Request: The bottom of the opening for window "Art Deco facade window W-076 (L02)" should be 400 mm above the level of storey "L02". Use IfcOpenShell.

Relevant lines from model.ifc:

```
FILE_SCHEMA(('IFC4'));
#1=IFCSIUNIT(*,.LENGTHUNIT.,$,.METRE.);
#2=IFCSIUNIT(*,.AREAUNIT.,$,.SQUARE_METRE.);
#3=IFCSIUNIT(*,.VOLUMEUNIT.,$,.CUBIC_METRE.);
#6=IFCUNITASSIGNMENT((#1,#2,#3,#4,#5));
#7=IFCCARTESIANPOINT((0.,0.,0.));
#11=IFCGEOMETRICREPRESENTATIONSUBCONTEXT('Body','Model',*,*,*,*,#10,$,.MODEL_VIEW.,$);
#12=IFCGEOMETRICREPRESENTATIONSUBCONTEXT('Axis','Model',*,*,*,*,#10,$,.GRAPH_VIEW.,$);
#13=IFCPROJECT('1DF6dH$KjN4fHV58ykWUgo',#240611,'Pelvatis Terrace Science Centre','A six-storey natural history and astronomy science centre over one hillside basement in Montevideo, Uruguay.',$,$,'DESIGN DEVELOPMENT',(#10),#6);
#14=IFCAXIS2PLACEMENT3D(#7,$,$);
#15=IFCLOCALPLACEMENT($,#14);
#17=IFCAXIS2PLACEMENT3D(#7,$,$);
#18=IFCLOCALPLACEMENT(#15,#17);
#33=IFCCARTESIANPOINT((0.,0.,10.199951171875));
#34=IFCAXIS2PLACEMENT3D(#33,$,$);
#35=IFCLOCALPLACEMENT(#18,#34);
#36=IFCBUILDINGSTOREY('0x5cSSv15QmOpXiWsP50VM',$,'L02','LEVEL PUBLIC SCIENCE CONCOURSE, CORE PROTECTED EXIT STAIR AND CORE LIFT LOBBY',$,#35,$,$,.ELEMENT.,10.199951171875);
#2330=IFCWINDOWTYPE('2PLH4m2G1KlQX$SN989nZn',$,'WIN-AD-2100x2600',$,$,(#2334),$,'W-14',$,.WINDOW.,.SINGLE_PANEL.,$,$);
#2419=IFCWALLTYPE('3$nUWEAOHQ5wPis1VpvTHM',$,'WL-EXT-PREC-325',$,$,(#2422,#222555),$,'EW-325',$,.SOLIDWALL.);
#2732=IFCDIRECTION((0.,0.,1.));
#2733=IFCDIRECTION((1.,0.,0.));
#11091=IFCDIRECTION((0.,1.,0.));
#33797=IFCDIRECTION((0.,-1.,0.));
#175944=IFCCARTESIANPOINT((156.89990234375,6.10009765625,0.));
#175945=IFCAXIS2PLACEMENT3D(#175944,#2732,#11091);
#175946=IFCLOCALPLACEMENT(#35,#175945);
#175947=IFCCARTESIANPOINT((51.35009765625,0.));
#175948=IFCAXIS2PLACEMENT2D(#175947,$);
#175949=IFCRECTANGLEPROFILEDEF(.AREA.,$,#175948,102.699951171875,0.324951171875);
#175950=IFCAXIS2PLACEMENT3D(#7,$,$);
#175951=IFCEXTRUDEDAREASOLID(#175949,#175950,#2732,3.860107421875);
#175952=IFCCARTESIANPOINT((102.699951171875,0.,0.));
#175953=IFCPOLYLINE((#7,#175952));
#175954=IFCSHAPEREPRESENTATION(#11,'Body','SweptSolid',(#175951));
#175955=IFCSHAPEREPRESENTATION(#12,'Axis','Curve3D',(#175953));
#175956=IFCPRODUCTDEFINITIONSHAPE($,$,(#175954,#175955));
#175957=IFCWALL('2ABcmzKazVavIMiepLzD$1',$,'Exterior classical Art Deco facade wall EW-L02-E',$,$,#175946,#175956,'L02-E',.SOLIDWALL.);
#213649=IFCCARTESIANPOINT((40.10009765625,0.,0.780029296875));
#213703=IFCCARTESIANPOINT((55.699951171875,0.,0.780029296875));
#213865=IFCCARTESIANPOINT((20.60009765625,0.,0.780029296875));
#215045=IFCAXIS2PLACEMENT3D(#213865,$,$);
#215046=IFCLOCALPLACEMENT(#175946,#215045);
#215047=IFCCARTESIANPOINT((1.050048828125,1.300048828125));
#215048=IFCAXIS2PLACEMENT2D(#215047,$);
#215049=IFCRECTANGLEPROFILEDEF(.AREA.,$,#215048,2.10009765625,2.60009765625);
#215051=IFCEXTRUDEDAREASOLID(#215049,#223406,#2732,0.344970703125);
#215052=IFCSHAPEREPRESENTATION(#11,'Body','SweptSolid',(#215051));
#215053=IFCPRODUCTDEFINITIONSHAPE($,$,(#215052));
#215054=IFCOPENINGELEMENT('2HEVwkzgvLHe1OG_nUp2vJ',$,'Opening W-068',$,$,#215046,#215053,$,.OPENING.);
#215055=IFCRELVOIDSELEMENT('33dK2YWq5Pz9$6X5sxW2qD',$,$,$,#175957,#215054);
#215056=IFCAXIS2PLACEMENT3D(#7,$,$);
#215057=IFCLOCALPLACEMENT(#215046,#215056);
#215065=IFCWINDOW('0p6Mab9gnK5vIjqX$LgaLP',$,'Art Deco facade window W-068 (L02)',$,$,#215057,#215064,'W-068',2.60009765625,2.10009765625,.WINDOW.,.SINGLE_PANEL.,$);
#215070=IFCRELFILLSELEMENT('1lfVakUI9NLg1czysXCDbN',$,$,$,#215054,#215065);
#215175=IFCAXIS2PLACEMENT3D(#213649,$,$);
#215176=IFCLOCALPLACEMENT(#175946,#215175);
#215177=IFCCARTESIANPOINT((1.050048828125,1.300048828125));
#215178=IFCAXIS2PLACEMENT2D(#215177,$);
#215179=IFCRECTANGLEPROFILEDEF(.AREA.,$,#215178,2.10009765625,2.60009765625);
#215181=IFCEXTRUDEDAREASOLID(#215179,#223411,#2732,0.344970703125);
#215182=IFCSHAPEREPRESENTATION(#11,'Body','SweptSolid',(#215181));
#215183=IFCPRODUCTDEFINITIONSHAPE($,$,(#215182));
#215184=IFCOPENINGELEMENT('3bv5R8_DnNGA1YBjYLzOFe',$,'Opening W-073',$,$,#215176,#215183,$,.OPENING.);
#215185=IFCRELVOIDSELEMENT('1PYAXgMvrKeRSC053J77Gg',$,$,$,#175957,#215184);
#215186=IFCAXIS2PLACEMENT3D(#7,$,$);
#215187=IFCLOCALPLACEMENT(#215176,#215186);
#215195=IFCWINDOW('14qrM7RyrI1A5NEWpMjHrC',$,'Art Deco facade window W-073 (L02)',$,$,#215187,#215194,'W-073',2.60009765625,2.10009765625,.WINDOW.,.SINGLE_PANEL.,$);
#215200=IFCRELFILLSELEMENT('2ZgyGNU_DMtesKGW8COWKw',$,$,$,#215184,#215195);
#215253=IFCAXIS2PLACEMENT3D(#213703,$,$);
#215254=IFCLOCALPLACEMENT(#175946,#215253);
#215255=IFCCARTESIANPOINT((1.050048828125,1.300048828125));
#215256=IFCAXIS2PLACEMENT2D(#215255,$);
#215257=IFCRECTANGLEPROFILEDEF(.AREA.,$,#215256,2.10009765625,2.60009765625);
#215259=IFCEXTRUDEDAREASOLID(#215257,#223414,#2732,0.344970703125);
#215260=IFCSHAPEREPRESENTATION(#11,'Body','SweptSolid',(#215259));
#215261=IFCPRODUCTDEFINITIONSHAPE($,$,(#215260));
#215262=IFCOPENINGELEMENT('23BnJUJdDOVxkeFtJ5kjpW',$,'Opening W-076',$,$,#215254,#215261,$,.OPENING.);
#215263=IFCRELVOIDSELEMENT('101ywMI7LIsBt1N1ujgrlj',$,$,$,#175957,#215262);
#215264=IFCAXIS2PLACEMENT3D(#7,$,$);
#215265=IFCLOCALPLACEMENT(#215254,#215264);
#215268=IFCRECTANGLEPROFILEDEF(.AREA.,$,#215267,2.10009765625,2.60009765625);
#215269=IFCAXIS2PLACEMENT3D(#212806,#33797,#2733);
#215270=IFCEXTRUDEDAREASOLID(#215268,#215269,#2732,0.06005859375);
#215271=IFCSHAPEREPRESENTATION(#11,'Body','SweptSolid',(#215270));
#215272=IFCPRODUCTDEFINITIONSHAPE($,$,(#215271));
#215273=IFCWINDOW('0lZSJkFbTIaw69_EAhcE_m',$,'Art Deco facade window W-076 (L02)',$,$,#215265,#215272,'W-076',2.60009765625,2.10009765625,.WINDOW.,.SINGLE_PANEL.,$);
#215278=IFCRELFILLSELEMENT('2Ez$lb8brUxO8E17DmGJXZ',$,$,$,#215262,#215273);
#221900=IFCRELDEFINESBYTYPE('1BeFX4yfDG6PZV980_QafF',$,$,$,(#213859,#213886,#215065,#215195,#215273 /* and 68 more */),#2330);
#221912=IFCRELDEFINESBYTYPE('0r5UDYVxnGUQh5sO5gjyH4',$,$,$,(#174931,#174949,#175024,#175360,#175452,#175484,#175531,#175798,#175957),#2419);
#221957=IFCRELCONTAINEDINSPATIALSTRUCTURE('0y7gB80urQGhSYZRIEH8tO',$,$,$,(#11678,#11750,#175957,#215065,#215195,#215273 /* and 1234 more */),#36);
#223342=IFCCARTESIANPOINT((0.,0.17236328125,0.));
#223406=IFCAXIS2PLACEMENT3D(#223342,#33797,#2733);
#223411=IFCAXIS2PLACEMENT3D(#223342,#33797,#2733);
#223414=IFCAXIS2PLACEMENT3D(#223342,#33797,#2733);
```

```python
import numpy as np
import ifcopenshell
import ifcopenshell.api.geometry
import ifcopenshell.geom
import ifcopenshell.util.element
import ifcopenshell.util.placement
import ifcopenshell.util.shape
import ifcopenshell.util.unit

model = ifcopenshell.open("model.ifc")
unit_scale = ifcopenshell.util.unit.calculate_unit_scale(model)

window = model.by_guid("0lZSJkFbTIaw69_EAhcE_m")
opening = window.FillsVoids[0].RelatingOpeningElement
storey = ifcopenshell.util.element.get_container(window, ifc_class="IfcBuildingStorey")
level = ifcopenshell.util.placement.get_local_placement(storey.ObjectPlacement)[2, 3]

# The opening's origin need not be at the sill, so measure its lowest point.
shape = ifcopenshell.geom.create_shape(ifcopenshell.geom.settings(), opening)
bottom = ifcopenshell.util.shape.get_shape_bottom_elevation(shape, shape.geometry) / unit_scale
dz = level + 0.4 - bottom

shift = np.array([0.0, 0.0, dz])
# The window is placed relative to its opening, so it follows when the opening moves.
matrix = ifcopenshell.util.placement.get_local_placement(opening.ObjectPlacement)
matrix[:3, 3] += shift
ifcopenshell.api.geometry.edit_object_placement(
    model, product=opening, matrix=matrix, is_si=False, should_transform_children=True
)

print(f"moved by {dz * unit_scale:+.3f} m")

model.write("model-out.ifc")
```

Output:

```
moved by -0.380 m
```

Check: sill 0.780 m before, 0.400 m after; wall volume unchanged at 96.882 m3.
